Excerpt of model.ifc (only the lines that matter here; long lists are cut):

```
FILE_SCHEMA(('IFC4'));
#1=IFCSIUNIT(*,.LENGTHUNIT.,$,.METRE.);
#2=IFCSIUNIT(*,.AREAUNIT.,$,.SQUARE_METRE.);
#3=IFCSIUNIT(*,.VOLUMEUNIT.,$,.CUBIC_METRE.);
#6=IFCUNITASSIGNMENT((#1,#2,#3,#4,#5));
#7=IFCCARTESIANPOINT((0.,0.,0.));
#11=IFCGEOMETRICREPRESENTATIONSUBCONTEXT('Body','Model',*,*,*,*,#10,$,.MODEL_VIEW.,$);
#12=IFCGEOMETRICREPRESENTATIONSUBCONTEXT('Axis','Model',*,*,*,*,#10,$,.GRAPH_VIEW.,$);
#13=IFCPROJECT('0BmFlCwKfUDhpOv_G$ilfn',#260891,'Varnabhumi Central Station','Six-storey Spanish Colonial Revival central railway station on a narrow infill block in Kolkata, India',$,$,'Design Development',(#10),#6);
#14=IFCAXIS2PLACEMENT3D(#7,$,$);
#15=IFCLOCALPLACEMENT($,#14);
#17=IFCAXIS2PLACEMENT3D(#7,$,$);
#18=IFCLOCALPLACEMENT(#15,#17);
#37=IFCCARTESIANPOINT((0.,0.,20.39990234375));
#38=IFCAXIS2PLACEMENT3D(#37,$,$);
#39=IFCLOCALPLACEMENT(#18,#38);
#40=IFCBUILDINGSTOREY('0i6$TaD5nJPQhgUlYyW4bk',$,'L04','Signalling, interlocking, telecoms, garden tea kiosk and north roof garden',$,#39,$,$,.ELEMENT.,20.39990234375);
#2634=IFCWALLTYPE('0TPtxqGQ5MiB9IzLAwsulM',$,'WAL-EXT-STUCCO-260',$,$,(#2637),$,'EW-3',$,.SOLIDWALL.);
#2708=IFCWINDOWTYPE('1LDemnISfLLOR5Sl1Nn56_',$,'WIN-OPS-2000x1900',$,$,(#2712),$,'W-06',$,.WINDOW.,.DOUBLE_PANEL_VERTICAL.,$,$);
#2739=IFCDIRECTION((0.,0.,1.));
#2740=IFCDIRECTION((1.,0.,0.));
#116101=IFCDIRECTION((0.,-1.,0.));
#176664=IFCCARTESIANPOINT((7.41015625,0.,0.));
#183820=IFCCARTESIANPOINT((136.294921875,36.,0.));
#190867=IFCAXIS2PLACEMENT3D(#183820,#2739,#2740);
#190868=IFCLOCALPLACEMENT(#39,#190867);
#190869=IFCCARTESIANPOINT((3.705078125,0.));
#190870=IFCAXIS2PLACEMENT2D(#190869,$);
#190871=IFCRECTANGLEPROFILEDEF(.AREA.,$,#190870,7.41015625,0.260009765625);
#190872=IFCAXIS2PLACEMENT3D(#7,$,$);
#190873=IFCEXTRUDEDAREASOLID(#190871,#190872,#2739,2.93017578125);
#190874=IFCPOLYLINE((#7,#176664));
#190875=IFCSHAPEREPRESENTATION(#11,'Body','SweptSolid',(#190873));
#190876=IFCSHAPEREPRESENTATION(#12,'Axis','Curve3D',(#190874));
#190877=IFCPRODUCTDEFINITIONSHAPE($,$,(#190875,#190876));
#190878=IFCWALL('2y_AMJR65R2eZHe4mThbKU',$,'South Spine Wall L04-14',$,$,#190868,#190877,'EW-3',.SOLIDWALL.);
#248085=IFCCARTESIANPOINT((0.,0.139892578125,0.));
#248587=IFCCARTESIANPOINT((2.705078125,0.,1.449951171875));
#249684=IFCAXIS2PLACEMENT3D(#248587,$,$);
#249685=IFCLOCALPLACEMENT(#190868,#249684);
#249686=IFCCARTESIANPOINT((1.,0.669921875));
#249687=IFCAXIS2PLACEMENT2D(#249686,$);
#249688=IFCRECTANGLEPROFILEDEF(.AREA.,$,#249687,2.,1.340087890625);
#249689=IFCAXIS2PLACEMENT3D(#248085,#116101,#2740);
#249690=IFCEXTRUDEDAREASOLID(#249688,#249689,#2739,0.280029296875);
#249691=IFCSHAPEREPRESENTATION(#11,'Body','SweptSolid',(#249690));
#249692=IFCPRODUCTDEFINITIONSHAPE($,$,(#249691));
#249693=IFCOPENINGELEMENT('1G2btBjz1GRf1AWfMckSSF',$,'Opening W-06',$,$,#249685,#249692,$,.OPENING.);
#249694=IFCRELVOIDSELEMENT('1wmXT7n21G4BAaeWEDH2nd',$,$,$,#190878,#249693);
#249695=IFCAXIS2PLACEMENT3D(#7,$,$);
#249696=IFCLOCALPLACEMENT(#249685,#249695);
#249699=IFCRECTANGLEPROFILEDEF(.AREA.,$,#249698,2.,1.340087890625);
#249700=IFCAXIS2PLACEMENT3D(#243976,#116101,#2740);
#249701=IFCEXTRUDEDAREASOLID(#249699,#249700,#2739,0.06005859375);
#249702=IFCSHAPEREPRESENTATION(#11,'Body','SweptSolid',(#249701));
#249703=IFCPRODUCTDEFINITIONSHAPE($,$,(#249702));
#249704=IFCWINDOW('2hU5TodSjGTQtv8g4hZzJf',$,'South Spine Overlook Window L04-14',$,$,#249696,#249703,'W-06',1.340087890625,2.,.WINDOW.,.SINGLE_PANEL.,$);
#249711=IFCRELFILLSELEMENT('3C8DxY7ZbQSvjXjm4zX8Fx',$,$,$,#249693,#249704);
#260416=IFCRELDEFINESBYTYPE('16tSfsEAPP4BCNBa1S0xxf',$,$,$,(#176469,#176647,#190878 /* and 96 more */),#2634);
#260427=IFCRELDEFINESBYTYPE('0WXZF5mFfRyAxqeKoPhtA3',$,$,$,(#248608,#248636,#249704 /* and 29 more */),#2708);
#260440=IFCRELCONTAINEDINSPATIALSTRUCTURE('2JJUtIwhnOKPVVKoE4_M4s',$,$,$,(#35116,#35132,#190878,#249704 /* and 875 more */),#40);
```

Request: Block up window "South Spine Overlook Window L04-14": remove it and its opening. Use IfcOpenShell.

```python
import ifcopenshell
import ifcopenshell.api.feature
import ifcopenshell.api.root
import ifcopenshell.geom
import ifcopenshell.util.shape

model = ifcopenshell.open("model.ifc")
settings = ifcopenshell.geom.settings()


def volume(element):
    """Net volume in cubic metres, openings subtracted."""
    shape = ifcopenshell.geom.create_shape(settings, element)
    return ifcopenshell.util.shape.get_volume(shape.geometry)


window = model.by_guid("2hU5TodSjGTQtv8g4hZzJf")
opening = window.FillsVoids[0].RelatingOpeningElement
wall = opening.VoidsElements[0].RelatingBuildingElement
before = volume(wall)

ifcopenshell.api.root.remove_product(model, product=window)
ifcopenshell.api.feature.remove_feature(model, feature=opening)

after = volume(wall)

print(f"wall volume {before:.3f} -> {after:.3f} m3")

model.write("model_rev.ifc")
```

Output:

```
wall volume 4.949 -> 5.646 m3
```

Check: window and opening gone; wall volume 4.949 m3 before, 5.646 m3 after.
